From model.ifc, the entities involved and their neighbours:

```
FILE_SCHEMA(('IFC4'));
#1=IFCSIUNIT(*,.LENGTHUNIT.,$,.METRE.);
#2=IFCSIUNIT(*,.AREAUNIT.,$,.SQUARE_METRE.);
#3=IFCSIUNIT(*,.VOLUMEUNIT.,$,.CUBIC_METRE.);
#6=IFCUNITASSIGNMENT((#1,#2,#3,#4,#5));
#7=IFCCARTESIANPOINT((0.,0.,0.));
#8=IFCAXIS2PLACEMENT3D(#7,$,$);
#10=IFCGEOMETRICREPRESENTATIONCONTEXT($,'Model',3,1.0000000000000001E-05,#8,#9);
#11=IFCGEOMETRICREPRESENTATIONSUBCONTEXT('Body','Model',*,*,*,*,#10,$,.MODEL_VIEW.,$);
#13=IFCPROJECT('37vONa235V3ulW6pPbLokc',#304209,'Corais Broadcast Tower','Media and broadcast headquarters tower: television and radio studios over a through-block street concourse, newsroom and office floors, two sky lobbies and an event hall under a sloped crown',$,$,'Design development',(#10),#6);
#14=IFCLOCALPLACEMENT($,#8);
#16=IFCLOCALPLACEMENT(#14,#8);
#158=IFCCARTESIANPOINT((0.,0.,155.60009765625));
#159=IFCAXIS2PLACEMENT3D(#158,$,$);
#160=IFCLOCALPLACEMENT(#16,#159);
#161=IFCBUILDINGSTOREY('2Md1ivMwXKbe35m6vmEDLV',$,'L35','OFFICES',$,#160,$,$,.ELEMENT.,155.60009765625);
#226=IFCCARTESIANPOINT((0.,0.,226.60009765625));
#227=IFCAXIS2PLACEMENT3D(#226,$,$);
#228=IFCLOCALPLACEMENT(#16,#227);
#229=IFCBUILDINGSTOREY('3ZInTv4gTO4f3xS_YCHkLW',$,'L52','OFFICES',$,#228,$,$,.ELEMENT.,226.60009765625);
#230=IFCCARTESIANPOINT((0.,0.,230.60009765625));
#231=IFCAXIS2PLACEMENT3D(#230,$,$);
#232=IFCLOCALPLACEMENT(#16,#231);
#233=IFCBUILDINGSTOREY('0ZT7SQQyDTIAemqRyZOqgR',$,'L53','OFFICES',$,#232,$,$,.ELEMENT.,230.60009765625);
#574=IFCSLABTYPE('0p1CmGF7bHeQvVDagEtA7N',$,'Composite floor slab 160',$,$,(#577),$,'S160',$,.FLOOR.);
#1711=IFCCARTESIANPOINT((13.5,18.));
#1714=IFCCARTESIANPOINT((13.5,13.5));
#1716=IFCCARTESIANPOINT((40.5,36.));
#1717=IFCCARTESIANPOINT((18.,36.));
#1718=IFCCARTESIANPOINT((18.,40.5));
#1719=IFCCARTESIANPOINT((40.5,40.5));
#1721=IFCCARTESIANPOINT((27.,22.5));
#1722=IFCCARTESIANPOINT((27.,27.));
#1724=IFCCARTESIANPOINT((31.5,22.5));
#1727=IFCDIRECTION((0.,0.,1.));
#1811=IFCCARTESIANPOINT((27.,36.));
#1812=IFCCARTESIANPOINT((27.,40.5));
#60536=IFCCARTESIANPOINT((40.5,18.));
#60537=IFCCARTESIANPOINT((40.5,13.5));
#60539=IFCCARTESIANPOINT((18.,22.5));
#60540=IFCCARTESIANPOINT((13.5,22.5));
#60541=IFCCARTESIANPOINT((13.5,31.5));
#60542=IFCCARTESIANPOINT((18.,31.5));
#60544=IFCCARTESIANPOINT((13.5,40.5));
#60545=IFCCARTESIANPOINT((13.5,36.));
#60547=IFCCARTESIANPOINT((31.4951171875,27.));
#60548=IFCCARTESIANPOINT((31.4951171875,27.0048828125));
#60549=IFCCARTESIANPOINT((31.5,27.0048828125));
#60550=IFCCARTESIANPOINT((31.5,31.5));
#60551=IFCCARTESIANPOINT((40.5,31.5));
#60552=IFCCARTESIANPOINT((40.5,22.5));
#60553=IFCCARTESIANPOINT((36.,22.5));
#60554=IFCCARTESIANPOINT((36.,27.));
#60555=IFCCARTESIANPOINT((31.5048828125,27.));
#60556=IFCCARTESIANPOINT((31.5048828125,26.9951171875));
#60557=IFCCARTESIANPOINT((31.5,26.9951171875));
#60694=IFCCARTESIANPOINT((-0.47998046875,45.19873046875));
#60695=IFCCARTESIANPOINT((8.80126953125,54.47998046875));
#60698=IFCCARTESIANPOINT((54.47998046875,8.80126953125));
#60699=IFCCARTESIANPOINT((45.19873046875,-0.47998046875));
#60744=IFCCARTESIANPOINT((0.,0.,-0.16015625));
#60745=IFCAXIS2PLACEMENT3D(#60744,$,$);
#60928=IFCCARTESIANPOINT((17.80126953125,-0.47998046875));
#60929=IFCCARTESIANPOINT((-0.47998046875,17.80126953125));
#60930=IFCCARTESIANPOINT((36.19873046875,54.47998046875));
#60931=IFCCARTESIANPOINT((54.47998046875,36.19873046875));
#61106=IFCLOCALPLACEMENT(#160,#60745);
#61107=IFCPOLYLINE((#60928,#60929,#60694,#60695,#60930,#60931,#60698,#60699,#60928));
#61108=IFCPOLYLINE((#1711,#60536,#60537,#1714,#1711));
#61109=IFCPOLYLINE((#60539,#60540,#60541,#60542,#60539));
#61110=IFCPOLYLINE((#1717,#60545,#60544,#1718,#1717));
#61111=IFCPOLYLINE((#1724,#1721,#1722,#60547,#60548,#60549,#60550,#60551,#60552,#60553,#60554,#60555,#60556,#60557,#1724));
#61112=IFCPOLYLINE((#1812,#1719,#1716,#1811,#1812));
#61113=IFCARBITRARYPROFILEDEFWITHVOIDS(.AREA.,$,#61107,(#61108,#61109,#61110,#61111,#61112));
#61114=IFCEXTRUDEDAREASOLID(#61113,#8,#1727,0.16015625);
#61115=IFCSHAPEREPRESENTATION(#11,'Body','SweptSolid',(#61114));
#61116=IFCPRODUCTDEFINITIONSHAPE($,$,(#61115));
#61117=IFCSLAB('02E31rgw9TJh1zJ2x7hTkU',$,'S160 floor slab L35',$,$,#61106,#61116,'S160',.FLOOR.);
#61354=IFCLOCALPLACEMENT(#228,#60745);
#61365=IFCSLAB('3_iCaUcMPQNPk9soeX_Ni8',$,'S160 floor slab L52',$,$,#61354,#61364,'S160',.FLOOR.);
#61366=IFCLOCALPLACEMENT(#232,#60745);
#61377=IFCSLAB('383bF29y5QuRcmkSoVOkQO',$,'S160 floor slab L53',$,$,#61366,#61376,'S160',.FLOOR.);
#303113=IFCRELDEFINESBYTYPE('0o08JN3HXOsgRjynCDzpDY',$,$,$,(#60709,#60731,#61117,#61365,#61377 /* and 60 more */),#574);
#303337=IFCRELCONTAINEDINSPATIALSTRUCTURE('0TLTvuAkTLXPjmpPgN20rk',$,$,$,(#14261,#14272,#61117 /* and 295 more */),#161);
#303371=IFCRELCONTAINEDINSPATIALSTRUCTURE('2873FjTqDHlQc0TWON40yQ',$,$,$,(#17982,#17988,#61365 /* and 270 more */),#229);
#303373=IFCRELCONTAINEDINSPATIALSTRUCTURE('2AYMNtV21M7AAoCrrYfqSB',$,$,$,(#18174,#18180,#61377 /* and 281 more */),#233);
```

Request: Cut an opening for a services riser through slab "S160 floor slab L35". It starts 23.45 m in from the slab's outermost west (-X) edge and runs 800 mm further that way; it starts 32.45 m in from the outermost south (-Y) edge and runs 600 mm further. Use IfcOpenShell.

```python
import numpy as np
import ifcopenshell
import ifcopenshell.api.feature
import ifcopenshell.api.geometry
import ifcopenshell.api.root
import ifcopenshell.geom
import ifcopenshell.util.placement
import ifcopenshell.util.representation
import ifcopenshell.util.shape
import ifcopenshell.util.unit

model = ifcopenshell.open("model.ifc")
unit_scale = ifcopenshell.util.unit.calculate_unit_scale(model)
settings = ifcopenshell.geom.settings()


def volume(element):
    """Net volume in cubic metres, openings subtracted."""
    shape = ifcopenshell.geom.create_shape(settings, element)
    return ifcopenshell.util.shape.get_volume(shape.geometry)


slab = model.by_guid("02E31rgw9TJh1zJ2x7hTkU")
before = volume(slab)

# Extent in the slab's own axes, in metres. The edges named are its -X and -Y sides.
slab_shape = ifcopenshell.geom.create_shape(settings, slab)
vertices = ifcopenshell.util.shape.get_vertices(slab_shape.geometry)
x_min, y_min, bottom = vertices.min(axis=0)
top = vertices[:, 2].max()

opening = ifcopenshell.api.root.create_entity(model, ifc_class="IfcOpeningElement", name="Services riser opening", predefined_type="OPENING")
context = ifcopenshell.util.representation.get_context(model, "Model", "Body", "MODEL_VIEW")
width, depth = 0.8, 0.6
outline = [(0.0, 0.0), (width, 0.0), (width, depth), (0.0, depth), (0.0, 0.0)]
# Overshoot both faces by 50 mm so the cut is clean.
shape = ifcopenshell.api.geometry.add_slab_representation(
    model, context=context, depth=top - bottom + 0.1, polyline=outline
)
ifcopenshell.api.geometry.assign_representation(model, product=opening, representation=shape)

matrix = ifcopenshell.util.placement.get_local_placement(slab.ObjectPlacement)
matrix[:, 3] = matrix @ np.append(np.array([x_min + 23.45, y_min + 32.45, bottom - 0.05]) / unit_scale, 1.0)
ifcopenshell.api.geometry.edit_object_placement(model, product=opening, matrix=matrix, is_si=False)
ifcopenshell.api.feature.add_feature(model, feature=opening, element=slab)

after = volume(slab)

print(f"slab volume {before:.3f} -> {after:.3f} m3")

model.write("model_v2.ifc")
```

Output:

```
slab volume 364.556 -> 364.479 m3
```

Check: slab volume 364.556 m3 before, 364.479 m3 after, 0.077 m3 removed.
